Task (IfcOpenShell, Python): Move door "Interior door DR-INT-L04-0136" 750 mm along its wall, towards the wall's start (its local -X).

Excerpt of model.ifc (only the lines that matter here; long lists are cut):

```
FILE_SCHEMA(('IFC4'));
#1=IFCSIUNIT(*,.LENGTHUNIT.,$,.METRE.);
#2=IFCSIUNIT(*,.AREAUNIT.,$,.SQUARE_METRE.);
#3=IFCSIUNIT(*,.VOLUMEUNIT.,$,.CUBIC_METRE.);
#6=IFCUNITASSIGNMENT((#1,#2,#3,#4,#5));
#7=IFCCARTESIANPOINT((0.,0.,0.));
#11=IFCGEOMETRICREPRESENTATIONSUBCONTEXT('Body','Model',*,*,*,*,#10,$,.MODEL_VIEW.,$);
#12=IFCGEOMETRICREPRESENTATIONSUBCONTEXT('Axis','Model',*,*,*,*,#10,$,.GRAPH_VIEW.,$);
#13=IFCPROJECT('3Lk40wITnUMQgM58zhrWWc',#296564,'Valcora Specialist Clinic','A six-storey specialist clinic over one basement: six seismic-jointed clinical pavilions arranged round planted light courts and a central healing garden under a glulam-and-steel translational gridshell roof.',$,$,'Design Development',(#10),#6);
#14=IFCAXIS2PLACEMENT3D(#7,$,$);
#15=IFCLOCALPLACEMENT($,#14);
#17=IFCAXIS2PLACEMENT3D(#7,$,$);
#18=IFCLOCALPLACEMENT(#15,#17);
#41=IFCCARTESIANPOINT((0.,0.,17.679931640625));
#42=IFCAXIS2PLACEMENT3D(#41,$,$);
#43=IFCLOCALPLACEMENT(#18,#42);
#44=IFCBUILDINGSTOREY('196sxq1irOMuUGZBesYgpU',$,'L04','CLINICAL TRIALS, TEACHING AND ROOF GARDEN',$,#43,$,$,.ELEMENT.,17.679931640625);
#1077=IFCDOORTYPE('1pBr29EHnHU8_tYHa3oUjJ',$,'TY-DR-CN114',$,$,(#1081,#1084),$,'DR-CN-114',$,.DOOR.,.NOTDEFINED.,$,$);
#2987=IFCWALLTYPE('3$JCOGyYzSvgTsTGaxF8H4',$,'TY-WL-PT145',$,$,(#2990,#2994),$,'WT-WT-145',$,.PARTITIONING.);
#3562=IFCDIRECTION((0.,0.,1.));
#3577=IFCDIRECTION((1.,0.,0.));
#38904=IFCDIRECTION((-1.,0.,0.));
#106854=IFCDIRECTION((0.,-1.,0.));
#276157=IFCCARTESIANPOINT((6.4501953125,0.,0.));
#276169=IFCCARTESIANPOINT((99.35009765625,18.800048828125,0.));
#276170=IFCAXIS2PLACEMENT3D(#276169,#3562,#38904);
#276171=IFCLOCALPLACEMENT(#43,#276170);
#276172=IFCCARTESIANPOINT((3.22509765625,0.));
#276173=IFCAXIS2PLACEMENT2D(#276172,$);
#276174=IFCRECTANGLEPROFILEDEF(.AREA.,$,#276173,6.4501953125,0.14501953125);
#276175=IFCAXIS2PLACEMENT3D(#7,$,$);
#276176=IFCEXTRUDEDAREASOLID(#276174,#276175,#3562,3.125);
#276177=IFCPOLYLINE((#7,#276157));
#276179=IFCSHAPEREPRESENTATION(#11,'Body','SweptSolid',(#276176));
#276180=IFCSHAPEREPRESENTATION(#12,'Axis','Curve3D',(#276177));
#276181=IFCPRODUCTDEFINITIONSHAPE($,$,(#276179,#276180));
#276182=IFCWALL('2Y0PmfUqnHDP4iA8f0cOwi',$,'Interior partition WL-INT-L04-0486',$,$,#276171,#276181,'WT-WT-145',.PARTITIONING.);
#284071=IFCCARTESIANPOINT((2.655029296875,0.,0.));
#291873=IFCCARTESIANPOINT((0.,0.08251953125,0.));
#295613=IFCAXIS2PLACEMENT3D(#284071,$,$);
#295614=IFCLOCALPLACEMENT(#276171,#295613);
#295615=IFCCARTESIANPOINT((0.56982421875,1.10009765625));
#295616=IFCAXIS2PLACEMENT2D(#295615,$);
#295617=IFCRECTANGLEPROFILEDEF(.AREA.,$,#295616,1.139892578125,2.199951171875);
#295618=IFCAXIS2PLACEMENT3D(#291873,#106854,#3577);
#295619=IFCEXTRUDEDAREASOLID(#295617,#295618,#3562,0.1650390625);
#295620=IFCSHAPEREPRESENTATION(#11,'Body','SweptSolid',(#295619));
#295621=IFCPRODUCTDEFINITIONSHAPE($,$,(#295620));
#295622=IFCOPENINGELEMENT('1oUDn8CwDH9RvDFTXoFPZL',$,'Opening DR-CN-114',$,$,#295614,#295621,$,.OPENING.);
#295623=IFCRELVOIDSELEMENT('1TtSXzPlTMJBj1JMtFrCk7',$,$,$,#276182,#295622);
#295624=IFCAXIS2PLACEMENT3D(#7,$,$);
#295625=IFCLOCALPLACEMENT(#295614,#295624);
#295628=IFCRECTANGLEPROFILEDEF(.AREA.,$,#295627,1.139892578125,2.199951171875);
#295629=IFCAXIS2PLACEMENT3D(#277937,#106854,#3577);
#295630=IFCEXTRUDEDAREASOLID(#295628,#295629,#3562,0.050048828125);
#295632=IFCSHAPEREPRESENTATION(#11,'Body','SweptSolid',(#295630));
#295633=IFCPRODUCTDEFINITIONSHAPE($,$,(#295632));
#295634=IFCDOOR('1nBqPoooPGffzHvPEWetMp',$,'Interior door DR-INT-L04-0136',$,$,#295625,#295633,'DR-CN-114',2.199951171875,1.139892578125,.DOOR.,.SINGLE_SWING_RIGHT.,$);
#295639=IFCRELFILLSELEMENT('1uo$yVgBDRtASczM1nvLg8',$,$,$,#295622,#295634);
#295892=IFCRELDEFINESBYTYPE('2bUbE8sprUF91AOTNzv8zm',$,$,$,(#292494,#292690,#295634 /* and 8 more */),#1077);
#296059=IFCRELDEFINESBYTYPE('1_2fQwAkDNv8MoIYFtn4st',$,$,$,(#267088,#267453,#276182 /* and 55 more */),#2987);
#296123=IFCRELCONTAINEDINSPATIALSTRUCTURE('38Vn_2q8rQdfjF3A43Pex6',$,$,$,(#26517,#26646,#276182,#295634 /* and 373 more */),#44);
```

```python
import ifcopenshell
import ifcopenshell.api.geometry
import ifcopenshell.util.placement
import ifcopenshell.util.unit

model = ifcopenshell.open("model.ifc")
unit_scale = ifcopenshell.util.unit.calculate_unit_scale(model)

door = model.by_guid("1nBqPoooPGffzHvPEWetMp")
opening = door.FillsVoids[0].RelatingOpeningElement
wall = opening.VoidsElements[0].RelatingBuildingElement

wall_matrix = ifcopenshell.util.placement.get_local_placement(wall.ObjectPlacement)
shift = wall_matrix[:3, 0] * -0.75 / unit_scale
before = ifcopenshell.util.placement.get_local_placement(door.ObjectPlacement)[:3, 3].copy()

# The door is placed relative to its opening, so it follows when the opening moves.
matrix = ifcopenshell.util.placement.get_local_placement(opening.ObjectPlacement)
matrix[:3, 3] += shift
ifcopenshell.api.geometry.edit_object_placement(
    model, product=opening, matrix=matrix, is_si=False, should_transform_children=True
)

after = ifcopenshell.util.placement.get_local_placement(door.ObjectPlacement)[:3, 3]
print("door moved by", (after - before).round(3) + 0.0)

model.write("model_v2.ifc")
```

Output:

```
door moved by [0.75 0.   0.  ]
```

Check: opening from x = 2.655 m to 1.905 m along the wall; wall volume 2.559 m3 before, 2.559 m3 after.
